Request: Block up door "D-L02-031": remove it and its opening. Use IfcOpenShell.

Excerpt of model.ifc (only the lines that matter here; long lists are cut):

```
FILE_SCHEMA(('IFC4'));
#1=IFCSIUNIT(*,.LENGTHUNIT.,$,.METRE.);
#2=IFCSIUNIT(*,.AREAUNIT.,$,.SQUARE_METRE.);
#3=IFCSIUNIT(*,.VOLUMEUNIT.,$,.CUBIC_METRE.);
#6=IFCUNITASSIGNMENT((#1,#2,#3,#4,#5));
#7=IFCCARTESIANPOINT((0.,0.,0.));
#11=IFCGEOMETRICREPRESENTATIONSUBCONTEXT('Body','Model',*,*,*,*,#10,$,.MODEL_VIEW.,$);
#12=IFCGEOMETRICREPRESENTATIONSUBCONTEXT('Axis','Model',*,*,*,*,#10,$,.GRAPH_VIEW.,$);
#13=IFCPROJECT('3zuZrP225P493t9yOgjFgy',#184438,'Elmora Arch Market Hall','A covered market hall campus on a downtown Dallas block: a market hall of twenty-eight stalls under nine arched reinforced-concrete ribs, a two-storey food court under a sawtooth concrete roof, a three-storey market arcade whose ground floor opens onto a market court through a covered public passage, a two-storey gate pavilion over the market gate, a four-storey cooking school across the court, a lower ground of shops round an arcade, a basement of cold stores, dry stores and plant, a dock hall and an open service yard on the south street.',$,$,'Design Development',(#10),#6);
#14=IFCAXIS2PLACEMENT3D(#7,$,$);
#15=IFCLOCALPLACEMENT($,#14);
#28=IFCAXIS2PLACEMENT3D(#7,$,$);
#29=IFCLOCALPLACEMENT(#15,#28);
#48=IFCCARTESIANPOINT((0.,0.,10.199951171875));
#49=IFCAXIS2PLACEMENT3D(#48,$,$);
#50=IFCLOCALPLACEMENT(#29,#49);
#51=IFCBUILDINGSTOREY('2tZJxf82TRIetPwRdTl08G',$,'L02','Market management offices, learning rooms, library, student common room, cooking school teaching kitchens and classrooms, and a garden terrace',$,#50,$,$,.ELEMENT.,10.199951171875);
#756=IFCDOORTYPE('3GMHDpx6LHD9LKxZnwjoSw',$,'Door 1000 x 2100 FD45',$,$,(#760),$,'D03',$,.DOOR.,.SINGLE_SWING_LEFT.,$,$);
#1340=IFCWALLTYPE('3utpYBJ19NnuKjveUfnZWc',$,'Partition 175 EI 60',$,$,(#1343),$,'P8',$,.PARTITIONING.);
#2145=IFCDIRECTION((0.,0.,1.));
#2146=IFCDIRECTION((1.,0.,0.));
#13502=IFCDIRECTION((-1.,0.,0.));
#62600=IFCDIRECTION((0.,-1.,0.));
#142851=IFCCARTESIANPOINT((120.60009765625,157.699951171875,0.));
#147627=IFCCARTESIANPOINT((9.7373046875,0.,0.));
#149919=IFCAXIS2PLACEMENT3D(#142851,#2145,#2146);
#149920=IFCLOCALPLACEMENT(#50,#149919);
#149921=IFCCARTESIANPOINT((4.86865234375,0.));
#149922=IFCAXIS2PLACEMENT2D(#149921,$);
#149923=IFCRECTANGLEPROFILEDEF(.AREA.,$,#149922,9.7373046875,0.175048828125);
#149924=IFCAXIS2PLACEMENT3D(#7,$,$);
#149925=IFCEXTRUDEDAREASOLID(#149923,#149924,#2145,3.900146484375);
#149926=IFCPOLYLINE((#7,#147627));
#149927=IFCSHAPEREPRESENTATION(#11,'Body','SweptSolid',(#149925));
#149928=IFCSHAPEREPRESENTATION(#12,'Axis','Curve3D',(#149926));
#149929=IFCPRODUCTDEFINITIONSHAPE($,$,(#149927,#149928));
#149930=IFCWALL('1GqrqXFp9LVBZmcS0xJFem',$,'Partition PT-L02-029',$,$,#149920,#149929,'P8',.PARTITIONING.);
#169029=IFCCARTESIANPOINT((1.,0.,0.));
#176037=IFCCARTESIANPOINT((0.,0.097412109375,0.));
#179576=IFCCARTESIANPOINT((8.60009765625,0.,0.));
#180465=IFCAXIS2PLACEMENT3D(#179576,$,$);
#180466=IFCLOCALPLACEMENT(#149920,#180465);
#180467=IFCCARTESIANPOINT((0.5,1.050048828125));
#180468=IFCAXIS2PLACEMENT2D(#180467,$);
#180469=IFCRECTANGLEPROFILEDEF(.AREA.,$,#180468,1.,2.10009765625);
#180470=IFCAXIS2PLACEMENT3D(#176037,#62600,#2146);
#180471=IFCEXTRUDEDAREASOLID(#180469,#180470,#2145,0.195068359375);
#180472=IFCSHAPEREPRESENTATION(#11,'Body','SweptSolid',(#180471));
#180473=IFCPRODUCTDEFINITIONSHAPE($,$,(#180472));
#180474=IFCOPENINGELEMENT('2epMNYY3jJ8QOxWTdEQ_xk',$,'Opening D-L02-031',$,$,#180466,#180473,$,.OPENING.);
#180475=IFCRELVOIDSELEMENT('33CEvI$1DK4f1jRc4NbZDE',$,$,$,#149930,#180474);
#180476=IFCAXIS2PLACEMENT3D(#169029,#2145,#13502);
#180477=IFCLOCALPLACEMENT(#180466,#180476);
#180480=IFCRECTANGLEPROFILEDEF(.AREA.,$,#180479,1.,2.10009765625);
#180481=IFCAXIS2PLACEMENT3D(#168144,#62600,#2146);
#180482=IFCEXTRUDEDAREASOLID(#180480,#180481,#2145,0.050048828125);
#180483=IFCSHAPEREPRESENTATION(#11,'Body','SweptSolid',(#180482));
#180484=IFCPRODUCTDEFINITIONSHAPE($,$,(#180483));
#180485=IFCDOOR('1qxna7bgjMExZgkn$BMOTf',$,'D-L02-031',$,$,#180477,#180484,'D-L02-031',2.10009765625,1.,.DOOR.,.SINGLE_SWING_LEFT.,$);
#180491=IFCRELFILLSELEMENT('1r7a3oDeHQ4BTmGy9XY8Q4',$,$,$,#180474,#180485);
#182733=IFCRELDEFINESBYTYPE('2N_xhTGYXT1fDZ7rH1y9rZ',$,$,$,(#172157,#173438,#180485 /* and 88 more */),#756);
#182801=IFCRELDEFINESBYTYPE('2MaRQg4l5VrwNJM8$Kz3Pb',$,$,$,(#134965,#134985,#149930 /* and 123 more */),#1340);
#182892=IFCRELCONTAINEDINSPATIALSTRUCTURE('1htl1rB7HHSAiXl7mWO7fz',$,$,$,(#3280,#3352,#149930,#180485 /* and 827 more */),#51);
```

```python
import ifcopenshell
import ifcopenshell.api.feature
import ifcopenshell.api.root
import ifcopenshell.geom
import ifcopenshell.util.shape

model = ifcopenshell.open("model.ifc")
settings = ifcopenshell.geom.settings()


def volume(element):
    """Net volume in cubic metres, openings subtracted."""
    shape = ifcopenshell.geom.create_shape(settings, element)
    return ifcopenshell.util.shape.get_volume(shape.geometry)


door = model.by_id(180485)
opening = door.FillsVoids[0].RelatingOpeningElement
wall = opening.VoidsElements[0].RelatingBuildingElement
before = volume(wall)

ifcopenshell.api.root.remove_product(model, product=door)
ifcopenshell.api.feature.remove_feature(model, feature=opening)

after = volume(wall)

print(f"wall volume {before:.3f} -> {after:.3f} m3")

model.write("model_v2.ifc")
```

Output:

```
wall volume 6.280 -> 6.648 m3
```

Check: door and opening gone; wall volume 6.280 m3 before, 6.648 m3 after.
